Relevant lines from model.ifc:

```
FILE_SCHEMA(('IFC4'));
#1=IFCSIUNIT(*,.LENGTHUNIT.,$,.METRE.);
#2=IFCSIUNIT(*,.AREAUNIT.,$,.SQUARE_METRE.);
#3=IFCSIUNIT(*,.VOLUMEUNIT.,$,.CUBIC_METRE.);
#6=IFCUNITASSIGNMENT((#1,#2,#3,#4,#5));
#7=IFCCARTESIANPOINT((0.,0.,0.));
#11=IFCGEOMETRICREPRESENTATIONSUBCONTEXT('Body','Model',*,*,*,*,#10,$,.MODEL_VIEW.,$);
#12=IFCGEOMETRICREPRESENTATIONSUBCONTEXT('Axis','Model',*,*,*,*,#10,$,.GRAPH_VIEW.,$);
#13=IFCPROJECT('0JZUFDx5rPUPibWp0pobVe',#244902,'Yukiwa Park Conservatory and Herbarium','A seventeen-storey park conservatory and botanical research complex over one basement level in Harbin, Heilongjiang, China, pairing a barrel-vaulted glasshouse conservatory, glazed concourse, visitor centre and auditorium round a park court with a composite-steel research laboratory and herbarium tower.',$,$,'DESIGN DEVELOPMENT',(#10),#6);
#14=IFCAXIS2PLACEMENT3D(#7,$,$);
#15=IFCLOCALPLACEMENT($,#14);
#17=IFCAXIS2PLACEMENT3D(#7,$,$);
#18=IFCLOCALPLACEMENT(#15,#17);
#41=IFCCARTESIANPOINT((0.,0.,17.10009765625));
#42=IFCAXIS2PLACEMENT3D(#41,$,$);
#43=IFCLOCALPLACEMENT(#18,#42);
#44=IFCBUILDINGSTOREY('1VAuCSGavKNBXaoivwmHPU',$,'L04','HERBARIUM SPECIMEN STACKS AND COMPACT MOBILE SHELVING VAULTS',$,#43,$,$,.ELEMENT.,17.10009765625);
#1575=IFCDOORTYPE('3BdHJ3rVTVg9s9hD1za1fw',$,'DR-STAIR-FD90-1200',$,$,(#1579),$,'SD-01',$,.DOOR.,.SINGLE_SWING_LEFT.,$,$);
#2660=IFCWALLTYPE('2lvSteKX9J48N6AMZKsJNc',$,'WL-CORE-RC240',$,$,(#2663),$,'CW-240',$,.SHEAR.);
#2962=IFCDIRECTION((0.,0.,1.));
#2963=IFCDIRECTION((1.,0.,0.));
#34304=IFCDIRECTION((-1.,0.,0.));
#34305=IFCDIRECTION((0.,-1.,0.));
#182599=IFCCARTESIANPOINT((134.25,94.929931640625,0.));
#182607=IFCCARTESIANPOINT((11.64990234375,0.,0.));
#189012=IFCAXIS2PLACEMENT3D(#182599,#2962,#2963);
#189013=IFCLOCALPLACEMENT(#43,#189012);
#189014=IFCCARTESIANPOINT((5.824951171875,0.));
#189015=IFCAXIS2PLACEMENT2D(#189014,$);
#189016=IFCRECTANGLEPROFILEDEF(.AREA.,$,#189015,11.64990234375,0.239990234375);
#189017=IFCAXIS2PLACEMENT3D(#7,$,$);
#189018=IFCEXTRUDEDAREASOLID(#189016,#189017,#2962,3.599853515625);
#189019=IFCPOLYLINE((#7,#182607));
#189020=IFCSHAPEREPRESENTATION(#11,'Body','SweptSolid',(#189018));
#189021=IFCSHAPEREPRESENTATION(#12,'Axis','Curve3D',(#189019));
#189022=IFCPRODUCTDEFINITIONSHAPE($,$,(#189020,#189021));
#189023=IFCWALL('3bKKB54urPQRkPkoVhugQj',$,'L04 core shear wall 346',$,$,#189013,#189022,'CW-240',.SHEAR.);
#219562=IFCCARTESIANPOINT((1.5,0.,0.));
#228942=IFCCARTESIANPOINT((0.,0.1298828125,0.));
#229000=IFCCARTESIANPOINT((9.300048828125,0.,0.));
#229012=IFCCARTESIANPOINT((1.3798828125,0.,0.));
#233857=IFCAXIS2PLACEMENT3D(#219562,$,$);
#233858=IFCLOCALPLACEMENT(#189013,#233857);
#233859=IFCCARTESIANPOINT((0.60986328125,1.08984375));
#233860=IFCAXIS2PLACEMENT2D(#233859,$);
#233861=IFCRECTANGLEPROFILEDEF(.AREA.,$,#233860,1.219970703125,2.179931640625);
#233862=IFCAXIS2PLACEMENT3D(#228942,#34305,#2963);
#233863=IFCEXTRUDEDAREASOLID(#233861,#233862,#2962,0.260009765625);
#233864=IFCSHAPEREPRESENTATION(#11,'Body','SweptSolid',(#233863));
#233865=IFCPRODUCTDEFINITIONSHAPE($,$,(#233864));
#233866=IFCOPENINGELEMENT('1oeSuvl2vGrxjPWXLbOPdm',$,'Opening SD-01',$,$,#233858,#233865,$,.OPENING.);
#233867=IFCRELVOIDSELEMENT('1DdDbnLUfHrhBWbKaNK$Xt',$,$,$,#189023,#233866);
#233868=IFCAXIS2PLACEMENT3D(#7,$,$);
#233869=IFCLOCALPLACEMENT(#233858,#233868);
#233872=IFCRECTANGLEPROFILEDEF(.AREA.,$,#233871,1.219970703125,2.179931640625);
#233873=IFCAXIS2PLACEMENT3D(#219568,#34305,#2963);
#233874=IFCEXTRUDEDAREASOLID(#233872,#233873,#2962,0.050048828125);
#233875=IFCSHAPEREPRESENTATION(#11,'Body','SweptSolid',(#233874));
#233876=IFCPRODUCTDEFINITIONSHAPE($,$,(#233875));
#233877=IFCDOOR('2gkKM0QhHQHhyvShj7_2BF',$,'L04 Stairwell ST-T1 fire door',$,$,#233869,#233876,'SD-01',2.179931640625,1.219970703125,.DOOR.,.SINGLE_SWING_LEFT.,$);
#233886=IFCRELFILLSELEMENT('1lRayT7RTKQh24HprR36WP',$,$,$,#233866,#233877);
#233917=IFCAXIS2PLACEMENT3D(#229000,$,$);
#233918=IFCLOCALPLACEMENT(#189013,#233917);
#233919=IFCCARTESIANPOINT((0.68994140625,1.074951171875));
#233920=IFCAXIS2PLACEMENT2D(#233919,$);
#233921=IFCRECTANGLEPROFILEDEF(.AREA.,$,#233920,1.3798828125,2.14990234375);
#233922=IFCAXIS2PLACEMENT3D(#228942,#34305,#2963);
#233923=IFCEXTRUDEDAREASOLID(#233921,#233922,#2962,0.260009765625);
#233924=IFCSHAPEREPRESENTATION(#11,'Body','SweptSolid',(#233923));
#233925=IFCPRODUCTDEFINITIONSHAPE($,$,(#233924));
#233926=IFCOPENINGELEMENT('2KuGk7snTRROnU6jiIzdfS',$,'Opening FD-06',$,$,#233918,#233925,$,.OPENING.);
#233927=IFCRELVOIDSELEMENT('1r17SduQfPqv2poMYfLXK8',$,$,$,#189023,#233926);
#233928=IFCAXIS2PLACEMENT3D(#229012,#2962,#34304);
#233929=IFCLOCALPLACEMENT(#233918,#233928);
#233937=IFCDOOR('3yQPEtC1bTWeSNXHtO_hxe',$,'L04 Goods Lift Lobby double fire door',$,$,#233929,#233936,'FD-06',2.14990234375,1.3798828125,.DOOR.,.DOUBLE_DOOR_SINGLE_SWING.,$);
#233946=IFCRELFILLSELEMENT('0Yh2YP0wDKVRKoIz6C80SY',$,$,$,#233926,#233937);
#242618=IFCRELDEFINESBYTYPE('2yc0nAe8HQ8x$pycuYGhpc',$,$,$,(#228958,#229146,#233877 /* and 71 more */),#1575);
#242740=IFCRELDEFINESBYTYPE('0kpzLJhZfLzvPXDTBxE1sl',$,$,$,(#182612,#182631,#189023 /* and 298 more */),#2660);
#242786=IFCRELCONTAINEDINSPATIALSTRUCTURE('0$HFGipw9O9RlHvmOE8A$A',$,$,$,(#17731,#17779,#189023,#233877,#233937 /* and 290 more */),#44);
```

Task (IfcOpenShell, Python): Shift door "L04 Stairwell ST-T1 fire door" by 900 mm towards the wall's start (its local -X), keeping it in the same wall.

```python
import ifcopenshell
import ifcopenshell.api.geometry
import ifcopenshell.util.placement

model = ifcopenshell.open("model.ifc")

door = model.by_guid("2gkKM0QhHQHhyvShj7_2BF")
opening = door.FillsVoids[0].RelatingOpeningElement
wall = opening.VoidsElements[0].RelatingBuildingElement

wall_matrix = ifcopenshell.util.placement.get_local_placement(wall.ObjectPlacement)
shift = wall_matrix[:3, 0] * -0.9
before = ifcopenshell.util.placement.get_local_placement(door.ObjectPlacement)[:3, 3].copy()

# The door is placed relative to its opening, so it follows when the opening moves.
matrix = ifcopenshell.util.placement.get_local_placement(opening.ObjectPlacement)
matrix[:3, 3] += shift
ifcopenshell.api.geometry.edit_object_placement(
    model, product=opening, matrix=matrix, is_si=False, should_transform_children=True
)

after = ifcopenshell.util.placement.get_local_placement(door.ObjectPlacement)[:3, 3]
print("door moved by", (after - before).round(3) + 0.0)

model.write("model_edited.ifc")
```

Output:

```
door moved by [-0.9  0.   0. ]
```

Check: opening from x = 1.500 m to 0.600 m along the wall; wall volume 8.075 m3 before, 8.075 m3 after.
